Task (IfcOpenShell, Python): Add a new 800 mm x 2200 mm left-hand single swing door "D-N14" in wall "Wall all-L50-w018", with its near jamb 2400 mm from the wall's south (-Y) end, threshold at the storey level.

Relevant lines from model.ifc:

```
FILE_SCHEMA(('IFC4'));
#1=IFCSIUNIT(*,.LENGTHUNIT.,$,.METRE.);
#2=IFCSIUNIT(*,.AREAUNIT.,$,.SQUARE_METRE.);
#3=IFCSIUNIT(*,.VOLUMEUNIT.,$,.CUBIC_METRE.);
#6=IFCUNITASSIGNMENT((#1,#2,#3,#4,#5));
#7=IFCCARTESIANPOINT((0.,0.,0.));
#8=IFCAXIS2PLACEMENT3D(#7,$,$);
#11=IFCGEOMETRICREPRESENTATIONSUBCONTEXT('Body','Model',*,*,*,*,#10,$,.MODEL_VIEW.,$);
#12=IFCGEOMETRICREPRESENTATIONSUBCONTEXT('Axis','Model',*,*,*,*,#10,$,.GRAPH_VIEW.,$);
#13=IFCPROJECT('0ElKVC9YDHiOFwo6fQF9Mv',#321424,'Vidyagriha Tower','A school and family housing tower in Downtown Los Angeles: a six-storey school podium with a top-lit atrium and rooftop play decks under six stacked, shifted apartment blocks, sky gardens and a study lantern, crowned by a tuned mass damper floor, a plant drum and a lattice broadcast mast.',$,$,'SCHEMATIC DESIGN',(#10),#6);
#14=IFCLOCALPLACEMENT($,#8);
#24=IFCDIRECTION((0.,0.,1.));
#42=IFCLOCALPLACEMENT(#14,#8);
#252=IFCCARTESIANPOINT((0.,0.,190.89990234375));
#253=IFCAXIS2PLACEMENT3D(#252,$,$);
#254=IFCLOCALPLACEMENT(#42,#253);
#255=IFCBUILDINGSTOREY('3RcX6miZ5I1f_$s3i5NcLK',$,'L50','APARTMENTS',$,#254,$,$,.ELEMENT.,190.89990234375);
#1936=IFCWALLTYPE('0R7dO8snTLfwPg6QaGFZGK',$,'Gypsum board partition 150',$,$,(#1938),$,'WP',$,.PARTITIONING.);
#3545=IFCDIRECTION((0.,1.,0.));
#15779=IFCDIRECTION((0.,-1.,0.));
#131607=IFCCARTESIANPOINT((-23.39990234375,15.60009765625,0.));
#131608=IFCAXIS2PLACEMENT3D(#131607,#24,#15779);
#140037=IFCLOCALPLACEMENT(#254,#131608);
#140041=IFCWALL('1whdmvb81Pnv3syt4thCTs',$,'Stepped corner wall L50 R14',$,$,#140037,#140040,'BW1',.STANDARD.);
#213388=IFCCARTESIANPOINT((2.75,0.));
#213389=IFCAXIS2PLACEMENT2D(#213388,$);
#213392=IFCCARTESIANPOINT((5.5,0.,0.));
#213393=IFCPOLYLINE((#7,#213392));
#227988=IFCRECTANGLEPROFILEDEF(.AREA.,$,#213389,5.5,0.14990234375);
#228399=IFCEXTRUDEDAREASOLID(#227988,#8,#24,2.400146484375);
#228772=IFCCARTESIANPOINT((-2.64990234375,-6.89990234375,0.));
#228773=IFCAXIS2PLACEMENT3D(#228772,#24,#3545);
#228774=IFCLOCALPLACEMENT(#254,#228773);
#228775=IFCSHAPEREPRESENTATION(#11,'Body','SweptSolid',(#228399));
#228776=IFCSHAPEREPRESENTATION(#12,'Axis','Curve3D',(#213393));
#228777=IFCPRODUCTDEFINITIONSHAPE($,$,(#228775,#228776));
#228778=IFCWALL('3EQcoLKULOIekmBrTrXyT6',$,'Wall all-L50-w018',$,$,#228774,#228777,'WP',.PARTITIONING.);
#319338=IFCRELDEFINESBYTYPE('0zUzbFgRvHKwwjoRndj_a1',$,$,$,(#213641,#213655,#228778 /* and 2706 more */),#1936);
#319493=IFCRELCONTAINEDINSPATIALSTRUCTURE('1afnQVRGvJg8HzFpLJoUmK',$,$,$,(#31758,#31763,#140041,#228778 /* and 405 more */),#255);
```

```python
import numpy as np
import ifcopenshell
import ifcopenshell.api.feature
import ifcopenshell.api.geometry
import ifcopenshell.api.root
import ifcopenshell.api.spatial
import ifcopenshell.geom
import ifcopenshell.util.element
import ifcopenshell.util.placement
import ifcopenshell.util.representation
import ifcopenshell.util.shape
import ifcopenshell.util.unit

model = ifcopenshell.open("model.ifc")
unit_scale = ifcopenshell.util.unit.calculate_unit_scale(model)
settings = ifcopenshell.geom.settings()


def volume(element):
    """Net volume in cubic metres, openings subtracted."""
    shape = ifcopenshell.geom.create_shape(settings, element)
    return ifcopenshell.util.shape.get_volume(shape.geometry)


wall = model.by_guid("3EQcoLKULOIekmBrTrXyT6")
storey = ifcopenshell.util.element.get_container(wall, ifc_class="IfcBuildingStorey")
context = ifcopenshell.util.representation.get_context(model, "Model", "Body", "MODEL_VIEW")
before = volume(wall)

width, height, from_end, sill = 0.8, 2.2, 2.4, 0.0  # metres

# The wall runs along its own X axis, and the end named is its -X end.
wall_shape = ifcopenshell.geom.create_shape(settings, wall)
x, y, z = ifcopenshell.util.shape.get_vertices(wall_shape.geometry).T
start = x.min() + from_end
face, thickness = float(y.min()), float(y.max() - y.min())
wall_matrix = ifcopenshell.util.placement.get_local_placement(wall.ObjectPlacement)
level = ifcopenshell.util.placement.get_local_placement(storey.ObjectPlacement)[2, 3]


def in_wall(x, y):
    """Placement at x, y metres in the wall's axes, at sill height."""
    matrix = wall_matrix.copy()
    matrix[:, 3] = wall_matrix @ np.array([x / unit_scale, y / unit_scale, 0.0, 1.0])
    matrix[2, 3] = level + sill / unit_scale
    return matrix


# Opening: a box that overshoots both wall faces by 50 mm.
opening = ifcopenshell.api.root.create_entity(model, ifc_class="IfcOpeningElement", predefined_type="OPENING")
box = ifcopenshell.api.geometry.add_wall_representation(
    model, context=context, length=width, height=height, thickness=thickness + 0.1
)
ifcopenshell.api.geometry.assign_representation(model, product=opening, representation=box)
ifcopenshell.api.geometry.edit_object_placement(model, product=opening, matrix=in_wall(start, face - 0.05), is_si=False)
ifcopenshell.api.feature.add_feature(model, feature=opening, element=wall)

door = ifcopenshell.api.root.create_entity(model, ifc_class="IfcDoor", name="D-N14", predefined_type="DOOR")
door.OverallWidth, door.OverallHeight = width / unit_scale, height / unit_scale
door.OperationType = "SINGLE_SWING_LEFT"
body = ifcopenshell.api.geometry.add_door_representation(
    model,
    context=context,
    overall_width=door.OverallWidth,
    overall_height=door.OverallHeight,
    operation_type="SINGLE_SWING_LEFT",
    lining_properties={"LiningDepth": thickness / unit_scale, "ThresholdDepth": thickness / unit_scale},
)
ifcopenshell.api.geometry.assign_representation(model, product=door, representation=body)
ifcopenshell.api.spatial.assign_container(model, products=[door], relating_structure=storey)
ifcopenshell.api.feature.add_filling(model, opening=opening, element=door)

# The lining spans the wall, so the door starts at the wall face.
ifcopenshell.api.geometry.edit_object_placement(model, product=door, matrix=in_wall(start, face), is_si=False)

after = volume(wall)

print(f"wall volume {before:.3f} -> {after:.3f} m3")

model.write("model-out.ifc")
```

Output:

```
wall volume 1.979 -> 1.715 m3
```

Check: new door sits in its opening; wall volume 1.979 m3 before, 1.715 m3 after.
